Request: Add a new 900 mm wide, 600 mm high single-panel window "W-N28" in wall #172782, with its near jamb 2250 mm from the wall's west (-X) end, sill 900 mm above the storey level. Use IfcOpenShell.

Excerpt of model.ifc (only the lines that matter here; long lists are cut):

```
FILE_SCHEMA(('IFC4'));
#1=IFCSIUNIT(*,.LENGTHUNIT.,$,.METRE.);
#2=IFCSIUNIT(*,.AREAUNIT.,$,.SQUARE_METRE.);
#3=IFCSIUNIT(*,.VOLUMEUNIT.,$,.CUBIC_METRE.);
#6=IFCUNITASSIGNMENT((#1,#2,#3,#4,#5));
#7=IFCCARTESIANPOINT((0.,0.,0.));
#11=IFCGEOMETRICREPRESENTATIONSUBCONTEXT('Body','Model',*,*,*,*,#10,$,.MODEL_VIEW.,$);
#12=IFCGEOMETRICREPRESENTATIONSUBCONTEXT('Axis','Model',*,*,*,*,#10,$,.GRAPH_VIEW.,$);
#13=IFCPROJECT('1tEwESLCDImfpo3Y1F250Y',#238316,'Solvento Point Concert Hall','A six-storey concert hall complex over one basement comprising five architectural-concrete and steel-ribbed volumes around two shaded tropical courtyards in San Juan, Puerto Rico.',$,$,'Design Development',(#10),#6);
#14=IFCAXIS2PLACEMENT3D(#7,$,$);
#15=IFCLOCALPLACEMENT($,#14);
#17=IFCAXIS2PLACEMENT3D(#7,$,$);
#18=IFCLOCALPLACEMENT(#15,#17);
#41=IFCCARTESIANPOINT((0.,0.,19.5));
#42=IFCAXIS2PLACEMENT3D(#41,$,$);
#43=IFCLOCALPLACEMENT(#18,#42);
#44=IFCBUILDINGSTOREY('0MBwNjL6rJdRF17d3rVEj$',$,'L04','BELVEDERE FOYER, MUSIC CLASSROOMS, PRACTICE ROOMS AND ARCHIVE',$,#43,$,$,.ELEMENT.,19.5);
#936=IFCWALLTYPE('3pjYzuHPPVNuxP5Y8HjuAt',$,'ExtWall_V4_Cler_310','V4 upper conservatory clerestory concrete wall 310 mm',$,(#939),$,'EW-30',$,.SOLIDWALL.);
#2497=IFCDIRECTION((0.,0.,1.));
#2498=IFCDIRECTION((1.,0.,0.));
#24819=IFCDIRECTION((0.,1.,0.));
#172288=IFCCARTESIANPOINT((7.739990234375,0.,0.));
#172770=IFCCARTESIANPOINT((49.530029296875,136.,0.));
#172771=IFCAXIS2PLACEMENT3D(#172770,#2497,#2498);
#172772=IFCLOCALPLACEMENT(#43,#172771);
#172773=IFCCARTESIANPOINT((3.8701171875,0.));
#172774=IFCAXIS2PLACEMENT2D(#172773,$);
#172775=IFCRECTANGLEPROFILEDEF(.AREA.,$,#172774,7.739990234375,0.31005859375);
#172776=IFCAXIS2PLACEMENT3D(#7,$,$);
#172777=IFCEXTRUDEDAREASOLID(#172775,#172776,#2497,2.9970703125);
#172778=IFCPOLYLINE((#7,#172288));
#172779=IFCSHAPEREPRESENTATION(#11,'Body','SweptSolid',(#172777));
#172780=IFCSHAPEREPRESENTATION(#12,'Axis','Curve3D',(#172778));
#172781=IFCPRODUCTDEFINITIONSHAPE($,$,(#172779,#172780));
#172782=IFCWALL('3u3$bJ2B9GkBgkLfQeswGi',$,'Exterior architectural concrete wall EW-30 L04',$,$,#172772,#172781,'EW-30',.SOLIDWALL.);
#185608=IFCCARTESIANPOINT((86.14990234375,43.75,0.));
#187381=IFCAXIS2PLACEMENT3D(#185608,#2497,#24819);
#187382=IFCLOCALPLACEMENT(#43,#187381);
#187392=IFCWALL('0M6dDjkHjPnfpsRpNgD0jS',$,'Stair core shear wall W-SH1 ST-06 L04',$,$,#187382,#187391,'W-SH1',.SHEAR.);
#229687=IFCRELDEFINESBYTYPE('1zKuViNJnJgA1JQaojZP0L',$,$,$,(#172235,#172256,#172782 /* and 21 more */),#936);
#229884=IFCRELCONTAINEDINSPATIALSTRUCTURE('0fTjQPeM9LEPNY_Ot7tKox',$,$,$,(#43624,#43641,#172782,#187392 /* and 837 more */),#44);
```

```python
import numpy as np
import ifcopenshell
import ifcopenshell.api.feature
import ifcopenshell.api.geometry
import ifcopenshell.api.root
import ifcopenshell.api.spatial
import ifcopenshell.geom
import ifcopenshell.util.element
import ifcopenshell.util.placement
import ifcopenshell.util.representation
import ifcopenshell.util.shape
import ifcopenshell.util.unit

model = ifcopenshell.open("model.ifc")
unit_scale = ifcopenshell.util.unit.calculate_unit_scale(model)
settings = ifcopenshell.geom.settings()


def volume(element):
    """Net volume in cubic metres, openings subtracted."""
    shape = ifcopenshell.geom.create_shape(settings, element)
    return ifcopenshell.util.shape.get_volume(shape.geometry)


wall = model.by_guid("3u3$bJ2B9GkBgkLfQeswGi")
storey = ifcopenshell.util.element.get_container(wall, ifc_class="IfcBuildingStorey")
context = ifcopenshell.util.representation.get_context(model, "Model", "Body", "MODEL_VIEW")
before = volume(wall)

width, height, from_end, sill = 0.9, 0.6, 2.25, 0.9  # metres

# The wall runs along its own X axis, and the end named is its -X end.
wall_shape = ifcopenshell.geom.create_shape(settings, wall)
x, y, z = ifcopenshell.util.shape.get_vertices(wall_shape.geometry).T
start = x.min() + from_end
face, thickness = float(y.min()), float(y.max() - y.min())
wall_matrix = ifcopenshell.util.placement.get_local_placement(wall.ObjectPlacement)
level = ifcopenshell.util.placement.get_local_placement(storey.ObjectPlacement)[2, 3]


def in_wall(x, y):
    """Placement at x, y metres in the wall's axes, at sill height."""
    matrix = wall_matrix.copy()
    matrix[:, 3] = wall_matrix @ np.array([x / unit_scale, y / unit_scale, 0.0, 1.0])
    matrix[2, 3] = level + sill / unit_scale
    return matrix


# Opening: a box that overshoots both wall faces by 50 mm.
opening = ifcopenshell.api.root.create_entity(model, ifc_class="IfcOpeningElement", predefined_type="OPENING")
box = ifcopenshell.api.geometry.add_wall_representation(
    model, context=context, length=width, height=height, thickness=thickness + 0.1
)
ifcopenshell.api.geometry.assign_representation(model, product=opening, representation=box)
ifcopenshell.api.geometry.edit_object_placement(model, product=opening, matrix=in_wall(start, face - 0.05), is_si=False)
ifcopenshell.api.feature.add_feature(model, feature=opening, element=wall)

window = ifcopenshell.api.root.create_entity(model, ifc_class="IfcWindow", name="W-N28", predefined_type="WINDOW")
window.OverallWidth, window.OverallHeight = width / unit_scale, height / unit_scale
window.PartitioningType = "SINGLE_PANEL"
body = ifcopenshell.api.geometry.add_window_representation(
    model,
    context=context,
    overall_width=window.OverallWidth,
    overall_height=window.OverallHeight,
    partition_type="SINGLE_PANEL",
)
ifcopenshell.api.geometry.assign_representation(model, product=window, representation=body)
ifcopenshell.api.spatial.assign_container(model, products=[window], relating_structure=storey)
ifcopenshell.api.feature.add_filling(model, opening=opening, element=window)

# Centre the window in the wall's thickness.
ifcopenshell.api.geometry.edit_object_placement(model, product=window, matrix=in_wall(start, face), is_si=False)
window_shape = ifcopenshell.geom.create_shape(settings, window)
depth = ifcopenshell.util.shape.get_vertices(window_shape.geometry)[:, 1]
offset = face + thickness / 2 - (depth.min() + depth.max()) / 2
ifcopenshell.api.geometry.edit_object_placement(model, product=window, matrix=in_wall(start, offset), is_si=False)

after = volume(wall)

print(f"wall volume {before:.3f} -> {after:.3f} m3")

model.write("model_rev.ifc")
```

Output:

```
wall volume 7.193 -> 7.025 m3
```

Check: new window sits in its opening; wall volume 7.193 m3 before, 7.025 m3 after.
